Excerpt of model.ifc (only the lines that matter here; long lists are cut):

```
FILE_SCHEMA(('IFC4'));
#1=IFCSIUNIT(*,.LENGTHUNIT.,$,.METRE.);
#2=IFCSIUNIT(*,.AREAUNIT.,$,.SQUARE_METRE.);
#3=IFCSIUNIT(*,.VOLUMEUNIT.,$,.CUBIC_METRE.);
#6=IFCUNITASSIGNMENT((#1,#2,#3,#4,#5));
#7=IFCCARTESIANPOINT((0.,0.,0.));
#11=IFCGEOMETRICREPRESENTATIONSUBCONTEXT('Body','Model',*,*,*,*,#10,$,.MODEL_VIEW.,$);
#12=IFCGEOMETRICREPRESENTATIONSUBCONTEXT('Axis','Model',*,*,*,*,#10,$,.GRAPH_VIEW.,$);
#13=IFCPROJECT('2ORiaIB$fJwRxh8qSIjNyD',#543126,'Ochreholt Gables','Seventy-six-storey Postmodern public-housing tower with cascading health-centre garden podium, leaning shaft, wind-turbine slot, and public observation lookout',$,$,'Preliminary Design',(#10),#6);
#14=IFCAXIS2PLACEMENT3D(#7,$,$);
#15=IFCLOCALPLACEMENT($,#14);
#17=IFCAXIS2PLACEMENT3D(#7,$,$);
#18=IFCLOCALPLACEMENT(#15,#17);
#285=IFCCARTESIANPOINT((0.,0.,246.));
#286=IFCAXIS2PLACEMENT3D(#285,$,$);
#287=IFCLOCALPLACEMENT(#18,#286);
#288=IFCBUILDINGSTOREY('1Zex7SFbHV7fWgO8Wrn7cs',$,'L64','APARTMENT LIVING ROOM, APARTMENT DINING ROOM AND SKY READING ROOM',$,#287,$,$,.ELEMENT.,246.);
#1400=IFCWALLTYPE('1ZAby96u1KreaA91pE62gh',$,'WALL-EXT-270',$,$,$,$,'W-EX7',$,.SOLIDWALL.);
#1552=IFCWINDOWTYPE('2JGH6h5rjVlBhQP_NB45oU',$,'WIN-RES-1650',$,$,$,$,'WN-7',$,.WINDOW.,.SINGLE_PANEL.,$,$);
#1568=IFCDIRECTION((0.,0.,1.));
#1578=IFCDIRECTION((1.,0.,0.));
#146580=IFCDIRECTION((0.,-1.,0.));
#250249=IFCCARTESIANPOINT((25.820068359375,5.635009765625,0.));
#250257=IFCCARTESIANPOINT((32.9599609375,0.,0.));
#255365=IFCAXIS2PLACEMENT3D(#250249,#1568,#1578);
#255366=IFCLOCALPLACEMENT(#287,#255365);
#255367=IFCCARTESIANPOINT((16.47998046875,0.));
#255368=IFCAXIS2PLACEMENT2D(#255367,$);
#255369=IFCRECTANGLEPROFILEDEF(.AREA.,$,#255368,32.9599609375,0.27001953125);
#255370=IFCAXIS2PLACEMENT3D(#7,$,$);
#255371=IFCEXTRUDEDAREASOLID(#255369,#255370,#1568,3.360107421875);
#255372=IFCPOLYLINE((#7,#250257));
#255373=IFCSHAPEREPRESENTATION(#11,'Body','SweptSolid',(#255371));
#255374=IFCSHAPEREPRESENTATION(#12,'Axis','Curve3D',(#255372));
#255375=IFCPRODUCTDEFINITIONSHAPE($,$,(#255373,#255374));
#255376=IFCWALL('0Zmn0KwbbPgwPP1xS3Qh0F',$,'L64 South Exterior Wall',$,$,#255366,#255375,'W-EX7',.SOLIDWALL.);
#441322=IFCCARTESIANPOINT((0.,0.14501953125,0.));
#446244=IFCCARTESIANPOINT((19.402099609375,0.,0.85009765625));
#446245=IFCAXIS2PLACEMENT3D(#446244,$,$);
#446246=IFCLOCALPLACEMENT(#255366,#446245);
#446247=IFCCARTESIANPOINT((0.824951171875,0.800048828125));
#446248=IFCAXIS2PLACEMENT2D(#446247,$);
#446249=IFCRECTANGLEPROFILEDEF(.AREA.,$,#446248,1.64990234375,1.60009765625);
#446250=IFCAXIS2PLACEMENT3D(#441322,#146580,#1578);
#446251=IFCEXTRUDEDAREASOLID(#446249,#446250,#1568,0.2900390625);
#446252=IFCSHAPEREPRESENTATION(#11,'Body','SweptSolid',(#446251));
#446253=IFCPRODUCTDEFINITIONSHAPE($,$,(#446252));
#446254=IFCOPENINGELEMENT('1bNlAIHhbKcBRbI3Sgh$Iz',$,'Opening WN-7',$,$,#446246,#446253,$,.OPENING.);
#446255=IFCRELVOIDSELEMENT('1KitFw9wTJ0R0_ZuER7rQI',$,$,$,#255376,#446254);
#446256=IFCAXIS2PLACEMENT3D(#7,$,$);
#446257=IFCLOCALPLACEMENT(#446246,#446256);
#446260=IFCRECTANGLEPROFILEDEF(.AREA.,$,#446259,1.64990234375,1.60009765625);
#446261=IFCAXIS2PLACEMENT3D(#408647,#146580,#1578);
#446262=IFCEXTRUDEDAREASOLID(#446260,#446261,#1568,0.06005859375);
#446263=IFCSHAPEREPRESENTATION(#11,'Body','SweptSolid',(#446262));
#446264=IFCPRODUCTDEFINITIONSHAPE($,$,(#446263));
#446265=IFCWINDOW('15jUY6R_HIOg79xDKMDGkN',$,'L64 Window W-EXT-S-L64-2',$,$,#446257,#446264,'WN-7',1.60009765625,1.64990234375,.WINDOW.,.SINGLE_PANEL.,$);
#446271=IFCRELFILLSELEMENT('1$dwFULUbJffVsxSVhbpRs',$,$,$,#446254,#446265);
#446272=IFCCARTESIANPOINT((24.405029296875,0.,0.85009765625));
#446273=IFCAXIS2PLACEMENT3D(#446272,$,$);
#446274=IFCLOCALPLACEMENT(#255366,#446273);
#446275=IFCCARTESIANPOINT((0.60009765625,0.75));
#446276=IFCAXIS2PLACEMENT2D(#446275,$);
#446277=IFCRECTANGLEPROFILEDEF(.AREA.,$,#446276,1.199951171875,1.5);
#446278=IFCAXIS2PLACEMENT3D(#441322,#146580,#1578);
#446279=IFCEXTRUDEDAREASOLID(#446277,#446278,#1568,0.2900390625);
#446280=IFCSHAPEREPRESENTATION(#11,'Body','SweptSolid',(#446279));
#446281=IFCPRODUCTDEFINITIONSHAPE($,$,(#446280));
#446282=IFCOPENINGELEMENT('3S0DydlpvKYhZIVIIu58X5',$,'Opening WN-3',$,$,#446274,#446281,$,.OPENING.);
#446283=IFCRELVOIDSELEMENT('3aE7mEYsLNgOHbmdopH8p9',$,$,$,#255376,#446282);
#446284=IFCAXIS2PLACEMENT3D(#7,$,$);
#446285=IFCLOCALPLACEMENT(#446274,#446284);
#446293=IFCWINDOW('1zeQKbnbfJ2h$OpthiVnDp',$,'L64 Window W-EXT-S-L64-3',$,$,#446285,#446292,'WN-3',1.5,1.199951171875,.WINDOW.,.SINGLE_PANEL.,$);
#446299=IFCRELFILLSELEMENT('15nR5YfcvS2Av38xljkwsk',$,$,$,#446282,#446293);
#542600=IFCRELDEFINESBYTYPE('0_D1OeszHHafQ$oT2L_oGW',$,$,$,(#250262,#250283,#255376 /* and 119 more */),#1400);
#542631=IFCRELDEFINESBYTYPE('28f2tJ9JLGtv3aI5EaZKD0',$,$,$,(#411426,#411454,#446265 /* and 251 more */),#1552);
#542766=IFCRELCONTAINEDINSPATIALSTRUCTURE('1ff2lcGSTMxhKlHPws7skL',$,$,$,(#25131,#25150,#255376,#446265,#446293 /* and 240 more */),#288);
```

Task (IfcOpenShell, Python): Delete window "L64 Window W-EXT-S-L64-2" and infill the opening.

```python
import ifcopenshell
import ifcopenshell.api.feature
import ifcopenshell.api.root
import ifcopenshell.geom
import ifcopenshell.util.shape

model = ifcopenshell.open("model.ifc")
settings = ifcopenshell.geom.settings()


def volume(element):
    """Net volume in cubic metres, openings subtracted."""
    shape = ifcopenshell.geom.create_shape(settings, element)
    return ifcopenshell.util.shape.get_volume(shape.geometry)


window = model.by_guid("15jUY6R_HIOg79xDKMDGkN")
opening = window.FillsVoids[0].RelatingOpeningElement
wall = opening.VoidsElements[0].RelatingBuildingElement
before = volume(wall)

ifcopenshell.api.root.remove_product(model, product=window)
ifcopenshell.api.feature.remove_feature(model, feature=opening)

after = volume(wall)

print(f"wall volume {before:.3f} -> {after:.3f} m3")

model.write("model-out.ifc")
```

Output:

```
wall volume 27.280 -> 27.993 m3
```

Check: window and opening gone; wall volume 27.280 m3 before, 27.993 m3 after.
